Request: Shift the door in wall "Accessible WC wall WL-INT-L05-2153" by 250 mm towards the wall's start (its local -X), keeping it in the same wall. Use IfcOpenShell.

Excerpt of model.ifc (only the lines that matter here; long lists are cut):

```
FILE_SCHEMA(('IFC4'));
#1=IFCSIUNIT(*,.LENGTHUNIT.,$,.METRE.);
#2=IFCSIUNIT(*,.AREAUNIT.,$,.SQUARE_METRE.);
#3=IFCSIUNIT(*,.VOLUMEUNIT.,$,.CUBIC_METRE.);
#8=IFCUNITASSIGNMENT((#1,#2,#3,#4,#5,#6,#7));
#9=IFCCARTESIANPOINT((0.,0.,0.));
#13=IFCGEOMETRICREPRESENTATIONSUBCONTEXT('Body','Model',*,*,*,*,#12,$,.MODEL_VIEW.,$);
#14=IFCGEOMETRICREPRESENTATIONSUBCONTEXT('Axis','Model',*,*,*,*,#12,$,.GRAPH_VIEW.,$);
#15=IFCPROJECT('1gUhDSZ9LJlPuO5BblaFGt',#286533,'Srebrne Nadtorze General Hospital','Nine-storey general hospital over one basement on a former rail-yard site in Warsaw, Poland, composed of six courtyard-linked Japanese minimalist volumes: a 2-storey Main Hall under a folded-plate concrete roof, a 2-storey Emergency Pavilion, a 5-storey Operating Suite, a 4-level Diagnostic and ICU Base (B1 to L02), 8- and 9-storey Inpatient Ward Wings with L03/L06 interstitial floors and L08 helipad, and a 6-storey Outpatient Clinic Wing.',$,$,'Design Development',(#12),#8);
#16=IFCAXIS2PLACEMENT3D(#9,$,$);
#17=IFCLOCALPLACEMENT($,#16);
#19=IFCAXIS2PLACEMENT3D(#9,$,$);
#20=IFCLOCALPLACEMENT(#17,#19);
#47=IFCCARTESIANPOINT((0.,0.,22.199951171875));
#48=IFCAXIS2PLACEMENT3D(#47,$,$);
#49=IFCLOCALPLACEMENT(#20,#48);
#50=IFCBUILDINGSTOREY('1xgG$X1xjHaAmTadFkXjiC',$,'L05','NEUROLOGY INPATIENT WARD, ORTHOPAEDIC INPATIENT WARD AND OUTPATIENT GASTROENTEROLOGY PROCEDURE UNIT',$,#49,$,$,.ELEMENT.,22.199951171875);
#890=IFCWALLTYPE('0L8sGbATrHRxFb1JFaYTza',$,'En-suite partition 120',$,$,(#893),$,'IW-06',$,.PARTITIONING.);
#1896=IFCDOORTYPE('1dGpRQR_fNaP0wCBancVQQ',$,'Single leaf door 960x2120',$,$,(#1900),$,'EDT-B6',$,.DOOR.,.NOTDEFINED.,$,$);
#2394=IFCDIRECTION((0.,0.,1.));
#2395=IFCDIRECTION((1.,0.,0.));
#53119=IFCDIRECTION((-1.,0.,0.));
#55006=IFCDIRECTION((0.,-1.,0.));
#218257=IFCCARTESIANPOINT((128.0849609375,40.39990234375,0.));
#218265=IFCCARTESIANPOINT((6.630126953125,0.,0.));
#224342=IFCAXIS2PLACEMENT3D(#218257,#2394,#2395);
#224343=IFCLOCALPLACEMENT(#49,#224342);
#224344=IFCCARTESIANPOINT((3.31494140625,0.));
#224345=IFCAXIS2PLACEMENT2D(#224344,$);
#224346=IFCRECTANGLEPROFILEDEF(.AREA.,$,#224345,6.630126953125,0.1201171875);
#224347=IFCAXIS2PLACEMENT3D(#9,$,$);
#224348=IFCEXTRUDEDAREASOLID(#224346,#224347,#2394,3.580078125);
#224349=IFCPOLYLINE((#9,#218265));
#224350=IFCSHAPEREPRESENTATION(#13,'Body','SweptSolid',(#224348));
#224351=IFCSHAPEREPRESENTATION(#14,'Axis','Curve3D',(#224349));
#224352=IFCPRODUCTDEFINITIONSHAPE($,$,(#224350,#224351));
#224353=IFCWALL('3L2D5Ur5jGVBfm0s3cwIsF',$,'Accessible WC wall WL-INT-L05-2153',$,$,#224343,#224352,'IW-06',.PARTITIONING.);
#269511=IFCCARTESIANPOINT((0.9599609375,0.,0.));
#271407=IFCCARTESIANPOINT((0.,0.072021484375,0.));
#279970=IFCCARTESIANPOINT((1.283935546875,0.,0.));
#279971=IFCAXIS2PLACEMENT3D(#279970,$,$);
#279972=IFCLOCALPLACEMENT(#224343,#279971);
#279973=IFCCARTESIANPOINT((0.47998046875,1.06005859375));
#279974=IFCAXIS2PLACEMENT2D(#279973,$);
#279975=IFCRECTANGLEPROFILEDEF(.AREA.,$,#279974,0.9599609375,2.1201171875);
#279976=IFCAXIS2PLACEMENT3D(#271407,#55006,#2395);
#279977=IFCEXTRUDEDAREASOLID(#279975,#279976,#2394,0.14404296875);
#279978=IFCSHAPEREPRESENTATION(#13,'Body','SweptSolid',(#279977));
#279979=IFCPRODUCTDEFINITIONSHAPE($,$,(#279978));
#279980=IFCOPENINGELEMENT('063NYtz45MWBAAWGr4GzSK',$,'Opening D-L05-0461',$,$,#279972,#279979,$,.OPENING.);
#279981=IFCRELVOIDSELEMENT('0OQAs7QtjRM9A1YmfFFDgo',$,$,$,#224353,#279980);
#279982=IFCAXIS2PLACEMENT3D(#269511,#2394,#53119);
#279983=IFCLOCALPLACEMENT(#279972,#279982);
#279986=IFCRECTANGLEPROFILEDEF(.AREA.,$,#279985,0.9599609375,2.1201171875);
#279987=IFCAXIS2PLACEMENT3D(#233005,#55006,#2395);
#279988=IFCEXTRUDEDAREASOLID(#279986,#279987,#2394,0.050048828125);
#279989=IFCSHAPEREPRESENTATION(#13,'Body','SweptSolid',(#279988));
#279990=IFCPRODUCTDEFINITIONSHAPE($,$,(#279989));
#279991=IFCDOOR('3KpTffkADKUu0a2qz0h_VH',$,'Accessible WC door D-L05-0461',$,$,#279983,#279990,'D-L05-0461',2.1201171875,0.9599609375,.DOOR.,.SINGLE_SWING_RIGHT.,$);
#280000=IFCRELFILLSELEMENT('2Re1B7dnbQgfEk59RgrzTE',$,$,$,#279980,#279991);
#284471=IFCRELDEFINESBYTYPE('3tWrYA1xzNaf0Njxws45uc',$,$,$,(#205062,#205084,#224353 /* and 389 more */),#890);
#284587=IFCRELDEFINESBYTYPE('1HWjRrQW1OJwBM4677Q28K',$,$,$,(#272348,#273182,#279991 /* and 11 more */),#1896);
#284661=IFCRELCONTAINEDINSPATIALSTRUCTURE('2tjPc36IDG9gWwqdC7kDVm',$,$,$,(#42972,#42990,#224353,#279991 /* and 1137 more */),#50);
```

```python
import ifcopenshell
import ifcopenshell.api.geometry
import ifcopenshell.util.placement
import ifcopenshell.util.unit

model = ifcopenshell.open("model.ifc")
unit_scale = ifcopenshell.util.unit.calculate_unit_scale(model)

door = model.by_guid("3KpTffkADKUu0a2qz0h_VH")
opening = door.FillsVoids[0].RelatingOpeningElement
wall = opening.VoidsElements[0].RelatingBuildingElement

wall_matrix = ifcopenshell.util.placement.get_local_placement(wall.ObjectPlacement)
shift = wall_matrix[:3, 0] * -0.25 / unit_scale
before = ifcopenshell.util.placement.get_local_placement(door.ObjectPlacement)[:3, 3].copy()

# The door is placed relative to its opening, so it follows when the opening moves.
matrix = ifcopenshell.util.placement.get_local_placement(opening.ObjectPlacement)
matrix[:3, 3] += shift
ifcopenshell.api.geometry.edit_object_placement(
    model, product=opening, matrix=matrix, is_si=False, should_transform_children=True
)

after = ifcopenshell.util.placement.get_local_placement(door.ObjectPlacement)[:3, 3]
print("door moved by", (after - before).round(3) + 0.0)

model.write("model_v2.ifc")
```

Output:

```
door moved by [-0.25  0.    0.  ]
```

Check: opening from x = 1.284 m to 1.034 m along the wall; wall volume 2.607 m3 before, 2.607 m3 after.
